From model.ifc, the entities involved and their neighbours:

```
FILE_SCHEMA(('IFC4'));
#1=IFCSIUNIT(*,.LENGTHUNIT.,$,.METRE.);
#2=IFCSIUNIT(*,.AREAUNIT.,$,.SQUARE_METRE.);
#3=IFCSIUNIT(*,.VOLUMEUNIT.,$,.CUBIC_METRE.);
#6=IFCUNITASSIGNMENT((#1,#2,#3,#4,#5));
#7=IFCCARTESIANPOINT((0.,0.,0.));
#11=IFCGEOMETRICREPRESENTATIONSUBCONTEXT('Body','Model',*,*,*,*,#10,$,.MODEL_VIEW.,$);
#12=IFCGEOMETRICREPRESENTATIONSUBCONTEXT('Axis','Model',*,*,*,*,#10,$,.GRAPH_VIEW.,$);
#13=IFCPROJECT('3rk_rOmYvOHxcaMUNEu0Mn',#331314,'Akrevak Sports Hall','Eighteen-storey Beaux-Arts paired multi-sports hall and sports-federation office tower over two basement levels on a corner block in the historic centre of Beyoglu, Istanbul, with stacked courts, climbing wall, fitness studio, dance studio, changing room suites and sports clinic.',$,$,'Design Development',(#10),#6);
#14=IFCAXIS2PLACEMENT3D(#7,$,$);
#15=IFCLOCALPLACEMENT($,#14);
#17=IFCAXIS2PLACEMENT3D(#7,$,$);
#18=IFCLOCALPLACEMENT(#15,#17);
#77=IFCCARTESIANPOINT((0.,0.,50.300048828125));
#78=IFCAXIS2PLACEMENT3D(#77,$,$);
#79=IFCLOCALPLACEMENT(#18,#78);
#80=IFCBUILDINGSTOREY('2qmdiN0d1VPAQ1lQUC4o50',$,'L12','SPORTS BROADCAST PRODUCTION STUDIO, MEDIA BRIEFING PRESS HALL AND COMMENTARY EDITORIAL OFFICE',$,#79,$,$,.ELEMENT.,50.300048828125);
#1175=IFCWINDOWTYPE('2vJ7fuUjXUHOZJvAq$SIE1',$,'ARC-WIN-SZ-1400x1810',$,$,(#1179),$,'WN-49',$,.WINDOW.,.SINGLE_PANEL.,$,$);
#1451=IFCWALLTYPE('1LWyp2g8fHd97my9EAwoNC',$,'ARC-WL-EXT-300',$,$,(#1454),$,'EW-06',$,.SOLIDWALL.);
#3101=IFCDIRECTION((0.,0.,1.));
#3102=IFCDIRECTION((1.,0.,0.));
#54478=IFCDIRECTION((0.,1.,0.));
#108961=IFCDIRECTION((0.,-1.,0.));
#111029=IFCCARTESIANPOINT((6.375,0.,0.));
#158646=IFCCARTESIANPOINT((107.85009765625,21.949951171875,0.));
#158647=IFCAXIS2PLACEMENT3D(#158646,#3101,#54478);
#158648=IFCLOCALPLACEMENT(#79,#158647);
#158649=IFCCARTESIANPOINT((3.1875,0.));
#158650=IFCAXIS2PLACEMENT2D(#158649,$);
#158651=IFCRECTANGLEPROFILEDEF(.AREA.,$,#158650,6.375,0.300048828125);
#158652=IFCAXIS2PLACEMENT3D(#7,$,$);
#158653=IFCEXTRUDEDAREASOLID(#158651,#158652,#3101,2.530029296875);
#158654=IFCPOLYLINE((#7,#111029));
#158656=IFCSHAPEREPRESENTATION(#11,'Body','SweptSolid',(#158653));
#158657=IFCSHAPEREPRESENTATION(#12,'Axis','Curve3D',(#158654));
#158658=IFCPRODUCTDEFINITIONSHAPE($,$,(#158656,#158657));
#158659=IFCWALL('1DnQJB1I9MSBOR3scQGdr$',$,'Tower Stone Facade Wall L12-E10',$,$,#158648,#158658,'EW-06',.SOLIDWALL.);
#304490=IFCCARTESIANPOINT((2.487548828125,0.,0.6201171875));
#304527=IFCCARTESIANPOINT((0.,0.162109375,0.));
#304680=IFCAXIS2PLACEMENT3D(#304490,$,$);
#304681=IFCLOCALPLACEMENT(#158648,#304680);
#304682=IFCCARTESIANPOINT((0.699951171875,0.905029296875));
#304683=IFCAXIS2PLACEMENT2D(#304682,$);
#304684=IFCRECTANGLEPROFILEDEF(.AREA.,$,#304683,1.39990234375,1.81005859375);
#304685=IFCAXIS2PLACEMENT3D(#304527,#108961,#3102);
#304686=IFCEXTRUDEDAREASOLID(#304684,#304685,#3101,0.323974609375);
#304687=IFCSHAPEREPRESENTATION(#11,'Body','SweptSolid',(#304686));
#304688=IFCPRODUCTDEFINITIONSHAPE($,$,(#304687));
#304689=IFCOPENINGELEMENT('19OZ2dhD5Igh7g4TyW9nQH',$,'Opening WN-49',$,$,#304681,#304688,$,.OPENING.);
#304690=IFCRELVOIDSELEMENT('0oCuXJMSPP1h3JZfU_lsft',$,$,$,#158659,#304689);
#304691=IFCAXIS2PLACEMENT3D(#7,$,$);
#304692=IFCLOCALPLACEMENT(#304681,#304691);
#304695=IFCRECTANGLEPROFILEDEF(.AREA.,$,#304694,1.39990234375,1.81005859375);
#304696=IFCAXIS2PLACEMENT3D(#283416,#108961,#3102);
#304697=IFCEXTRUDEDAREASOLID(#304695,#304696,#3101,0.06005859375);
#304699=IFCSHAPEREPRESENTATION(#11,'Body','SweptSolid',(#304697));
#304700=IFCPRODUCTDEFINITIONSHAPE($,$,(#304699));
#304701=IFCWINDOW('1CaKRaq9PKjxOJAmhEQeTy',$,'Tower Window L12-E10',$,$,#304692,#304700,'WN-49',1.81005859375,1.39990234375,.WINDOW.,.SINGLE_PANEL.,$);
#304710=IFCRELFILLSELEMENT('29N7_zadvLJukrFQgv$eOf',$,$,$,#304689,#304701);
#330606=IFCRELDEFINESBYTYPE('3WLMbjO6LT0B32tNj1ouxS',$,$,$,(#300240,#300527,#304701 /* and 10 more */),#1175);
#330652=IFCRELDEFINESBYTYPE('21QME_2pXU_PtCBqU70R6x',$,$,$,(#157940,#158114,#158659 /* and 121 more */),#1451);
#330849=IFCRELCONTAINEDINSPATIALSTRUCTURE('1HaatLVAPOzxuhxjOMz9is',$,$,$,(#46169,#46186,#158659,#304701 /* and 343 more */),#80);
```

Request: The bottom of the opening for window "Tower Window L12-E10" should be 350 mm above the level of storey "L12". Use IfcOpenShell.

```python
import numpy as np
import ifcopenshell
import ifcopenshell.api.geometry
import ifcopenshell.geom
import ifcopenshell.util.element
import ifcopenshell.util.placement
import ifcopenshell.util.shape
import ifcopenshell.util.unit

model = ifcopenshell.open("model.ifc")
unit_scale = ifcopenshell.util.unit.calculate_unit_scale(model)

window = model.by_guid("1CaKRaq9PKjxOJAmhEQeTy")
opening = window.FillsVoids[0].RelatingOpeningElement
storey = ifcopenshell.util.element.get_container(window, ifc_class="IfcBuildingStorey")
level = ifcopenshell.util.placement.get_local_placement(storey.ObjectPlacement)[2, 3]

# The opening's origin need not be at the sill, so measure its lowest point.
shape = ifcopenshell.geom.create_shape(ifcopenshell.geom.settings(), opening)
bottom = ifcopenshell.util.shape.get_shape_bottom_elevation(shape, shape.geometry) / unit_scale
dz = level + 0.35 - bottom

shift = np.array([0.0, 0.0, dz])
# The window is placed relative to its opening, so it follows when the opening moves.
matrix = ifcopenshell.util.placement.get_local_placement(opening.ObjectPlacement)
matrix[:3, 3] += shift
ifcopenshell.api.geometry.edit_object_placement(
    model, product=opening, matrix=matrix, is_si=False, should_transform_children=True
)

print(f"moved by {dz * unit_scale:+.3f} m")

model.write("model_v2.ifc")
```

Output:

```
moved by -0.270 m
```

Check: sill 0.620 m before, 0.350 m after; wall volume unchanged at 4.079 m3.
